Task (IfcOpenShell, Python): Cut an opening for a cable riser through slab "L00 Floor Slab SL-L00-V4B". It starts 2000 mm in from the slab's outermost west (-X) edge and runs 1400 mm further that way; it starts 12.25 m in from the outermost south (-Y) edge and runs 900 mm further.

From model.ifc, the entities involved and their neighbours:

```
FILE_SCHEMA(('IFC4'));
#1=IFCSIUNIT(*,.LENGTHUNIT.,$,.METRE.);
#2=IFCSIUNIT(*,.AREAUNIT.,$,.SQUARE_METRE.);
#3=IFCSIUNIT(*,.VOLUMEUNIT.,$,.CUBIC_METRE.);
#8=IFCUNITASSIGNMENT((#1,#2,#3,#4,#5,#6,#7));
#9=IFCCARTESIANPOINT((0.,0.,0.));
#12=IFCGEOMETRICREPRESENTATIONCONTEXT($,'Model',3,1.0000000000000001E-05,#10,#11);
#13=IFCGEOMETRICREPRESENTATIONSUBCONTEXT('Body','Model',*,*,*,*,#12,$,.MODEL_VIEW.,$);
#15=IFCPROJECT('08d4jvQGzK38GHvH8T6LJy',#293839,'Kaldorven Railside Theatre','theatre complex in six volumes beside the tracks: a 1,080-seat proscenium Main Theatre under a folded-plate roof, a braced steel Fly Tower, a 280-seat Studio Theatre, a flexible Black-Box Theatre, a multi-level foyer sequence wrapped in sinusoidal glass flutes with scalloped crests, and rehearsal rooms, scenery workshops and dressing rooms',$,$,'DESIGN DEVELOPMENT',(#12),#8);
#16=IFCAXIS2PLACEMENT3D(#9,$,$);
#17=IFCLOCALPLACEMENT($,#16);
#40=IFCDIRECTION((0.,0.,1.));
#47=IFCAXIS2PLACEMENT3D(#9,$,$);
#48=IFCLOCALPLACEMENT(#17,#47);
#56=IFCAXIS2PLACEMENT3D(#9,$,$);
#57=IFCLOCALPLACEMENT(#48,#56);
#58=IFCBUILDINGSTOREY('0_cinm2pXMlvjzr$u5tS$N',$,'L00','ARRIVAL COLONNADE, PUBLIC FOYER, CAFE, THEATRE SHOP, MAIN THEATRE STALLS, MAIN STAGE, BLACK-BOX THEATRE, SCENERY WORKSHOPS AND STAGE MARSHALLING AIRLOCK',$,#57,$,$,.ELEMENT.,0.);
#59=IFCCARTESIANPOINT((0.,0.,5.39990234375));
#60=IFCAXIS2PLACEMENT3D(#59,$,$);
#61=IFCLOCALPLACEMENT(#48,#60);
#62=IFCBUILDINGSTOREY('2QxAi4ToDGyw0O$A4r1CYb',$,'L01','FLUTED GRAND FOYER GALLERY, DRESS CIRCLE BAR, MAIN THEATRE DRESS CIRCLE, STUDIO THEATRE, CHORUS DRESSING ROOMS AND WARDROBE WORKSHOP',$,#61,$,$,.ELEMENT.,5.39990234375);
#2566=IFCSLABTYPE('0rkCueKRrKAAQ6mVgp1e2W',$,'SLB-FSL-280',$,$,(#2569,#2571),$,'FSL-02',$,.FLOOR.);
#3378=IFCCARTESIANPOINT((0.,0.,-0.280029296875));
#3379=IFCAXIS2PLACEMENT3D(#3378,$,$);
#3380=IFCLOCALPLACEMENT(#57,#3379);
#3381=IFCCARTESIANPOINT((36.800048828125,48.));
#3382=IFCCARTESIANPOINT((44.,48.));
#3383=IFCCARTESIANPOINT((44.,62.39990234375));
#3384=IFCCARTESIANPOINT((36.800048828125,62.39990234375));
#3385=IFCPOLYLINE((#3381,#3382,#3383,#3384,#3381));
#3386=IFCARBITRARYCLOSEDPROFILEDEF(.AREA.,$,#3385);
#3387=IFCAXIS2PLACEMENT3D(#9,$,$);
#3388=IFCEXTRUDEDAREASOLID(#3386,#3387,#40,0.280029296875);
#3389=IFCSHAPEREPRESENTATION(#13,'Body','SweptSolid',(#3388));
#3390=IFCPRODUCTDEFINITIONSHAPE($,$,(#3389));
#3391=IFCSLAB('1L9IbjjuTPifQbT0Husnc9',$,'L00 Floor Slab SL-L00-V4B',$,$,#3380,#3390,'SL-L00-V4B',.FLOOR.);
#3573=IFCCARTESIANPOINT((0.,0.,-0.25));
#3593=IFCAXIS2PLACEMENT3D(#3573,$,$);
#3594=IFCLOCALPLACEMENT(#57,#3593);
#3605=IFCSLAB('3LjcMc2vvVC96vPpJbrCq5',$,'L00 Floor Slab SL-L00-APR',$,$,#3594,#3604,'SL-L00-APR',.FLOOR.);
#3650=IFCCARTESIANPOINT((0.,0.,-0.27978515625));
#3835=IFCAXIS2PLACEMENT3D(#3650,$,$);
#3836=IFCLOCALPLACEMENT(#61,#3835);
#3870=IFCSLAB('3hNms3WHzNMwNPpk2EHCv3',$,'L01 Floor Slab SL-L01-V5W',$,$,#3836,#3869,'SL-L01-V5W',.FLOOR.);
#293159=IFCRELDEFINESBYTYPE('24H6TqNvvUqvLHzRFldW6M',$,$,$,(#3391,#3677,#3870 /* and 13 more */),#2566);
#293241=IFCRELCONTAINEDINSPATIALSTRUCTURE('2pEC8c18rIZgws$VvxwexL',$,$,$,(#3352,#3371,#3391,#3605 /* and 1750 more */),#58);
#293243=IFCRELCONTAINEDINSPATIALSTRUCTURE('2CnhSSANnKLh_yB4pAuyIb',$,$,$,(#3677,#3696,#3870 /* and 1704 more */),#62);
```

```python
import numpy as np
import ifcopenshell
import ifcopenshell.api.feature
import ifcopenshell.api.geometry
import ifcopenshell.api.root
import ifcopenshell.geom
import ifcopenshell.util.placement
import ifcopenshell.util.representation
import ifcopenshell.util.shape
import ifcopenshell.util.unit

model = ifcopenshell.open("model.ifc")
unit_scale = ifcopenshell.util.unit.calculate_unit_scale(model)
settings = ifcopenshell.geom.settings()


def volume(element):
    """Net volume in cubic metres, openings subtracted."""
    shape = ifcopenshell.geom.create_shape(settings, element)
    return ifcopenshell.util.shape.get_volume(shape.geometry)


slab = model.by_guid("1L9IbjjuTPifQbT0Husnc9")
before = volume(slab)

# Extent in the slab's own axes, in metres. The edges named are its -X and -Y sides.
slab_shape = ifcopenshell.geom.create_shape(settings, slab)
vertices = ifcopenshell.util.shape.get_vertices(slab_shape.geometry)
x_min, y_min, bottom = vertices.min(axis=0)
top = vertices[:, 2].max()

opening = ifcopenshell.api.root.create_entity(model, ifc_class="IfcOpeningElement", name="Cable riser opening", predefined_type="OPENING")
context = ifcopenshell.util.representation.get_context(model, "Model", "Body", "MODEL_VIEW")
width, depth = 1.4, 0.9
outline = [(0.0, 0.0), (width, 0.0), (width, depth), (0.0, depth), (0.0, 0.0)]
# Overshoot both faces by 50 mm so the cut is clean.
shape = ifcopenshell.api.geometry.add_slab_representation(
    model, context=context, depth=top - bottom + 0.1, polyline=outline
)
ifcopenshell.api.geometry.assign_representation(model, product=opening, representation=shape)

matrix = ifcopenshell.util.placement.get_local_placement(slab.ObjectPlacement)
matrix[:, 3] = matrix @ np.append(np.array([x_min + 2, y_min + 12.25, bottom - 0.05]) / unit_scale, 1.0)
ifcopenshell.api.geometry.edit_object_placement(model, product=opening, matrix=matrix, is_si=False)
ifcopenshell.api.feature.add_feature(model, feature=opening, element=slab)

after = volume(slab)

print(f"slab volume {before:.3f} -> {after:.3f} m3")

model.write("model_edited.ifc")
```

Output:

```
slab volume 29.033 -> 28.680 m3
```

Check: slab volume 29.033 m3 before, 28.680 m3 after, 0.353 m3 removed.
